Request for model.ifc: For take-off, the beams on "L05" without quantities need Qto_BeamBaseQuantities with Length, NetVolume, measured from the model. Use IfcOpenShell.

First a look at what the model holds.

```python
import ifcopenshell
import ifcopenshell.util.element
import ifcopenshell.util.unit

model = ifcopenshell.open("model.ifc")
print(model.schema)
for unit_type in ("LENGTHUNIT", "AREAUNIT", "VOLUMEUNIT"):
    print(unit_type, ifcopenshell.util.unit.calculate_unit_scale(model, unit_type))
storey = next(s for s in model.by_type("IfcBuildingStorey") if s.Name == "L05")
beams = [e for e in ifcopenshell.util.element.get_decomposition(storey) if e.is_a("IfcBeam")]
for e in sorted(beams, key=lambda e: e.id()):
    print(e.id(), e.is_a(), e.Name, list(ifcopenshell.util.element.get_psets(e, qtos_only=True)), sep=" | ")
```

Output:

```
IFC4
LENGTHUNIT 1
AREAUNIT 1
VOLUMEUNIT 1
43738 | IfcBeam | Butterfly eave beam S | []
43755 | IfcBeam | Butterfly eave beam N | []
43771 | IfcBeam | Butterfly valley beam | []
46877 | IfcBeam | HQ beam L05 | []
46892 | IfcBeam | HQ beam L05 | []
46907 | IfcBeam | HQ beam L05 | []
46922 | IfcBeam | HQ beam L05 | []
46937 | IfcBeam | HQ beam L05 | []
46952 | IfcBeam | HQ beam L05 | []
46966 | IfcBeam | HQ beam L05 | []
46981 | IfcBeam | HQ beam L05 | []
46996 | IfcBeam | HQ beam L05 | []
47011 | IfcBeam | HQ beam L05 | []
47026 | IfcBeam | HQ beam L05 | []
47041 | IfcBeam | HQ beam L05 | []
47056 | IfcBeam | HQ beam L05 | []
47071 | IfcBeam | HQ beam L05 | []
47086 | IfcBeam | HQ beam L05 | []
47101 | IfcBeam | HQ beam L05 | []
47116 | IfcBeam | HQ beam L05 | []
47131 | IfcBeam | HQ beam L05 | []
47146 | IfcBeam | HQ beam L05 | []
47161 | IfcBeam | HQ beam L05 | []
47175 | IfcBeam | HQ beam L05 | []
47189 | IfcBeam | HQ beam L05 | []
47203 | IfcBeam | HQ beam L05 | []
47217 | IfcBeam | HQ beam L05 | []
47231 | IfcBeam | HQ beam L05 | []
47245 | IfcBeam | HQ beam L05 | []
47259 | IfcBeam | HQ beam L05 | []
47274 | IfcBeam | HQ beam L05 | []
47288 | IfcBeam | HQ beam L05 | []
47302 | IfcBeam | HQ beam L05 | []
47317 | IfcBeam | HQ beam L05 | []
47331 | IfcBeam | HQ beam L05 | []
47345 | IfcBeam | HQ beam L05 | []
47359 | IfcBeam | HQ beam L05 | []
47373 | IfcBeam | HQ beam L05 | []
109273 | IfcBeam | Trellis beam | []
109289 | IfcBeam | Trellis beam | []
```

```python
import ifcopenshell
import ifcopenshell.api.pset
import ifcopenshell.geom
import ifcopenshell.util.element
import ifcopenshell.util.shape
import ifcopenshell.util.unit

model = ifcopenshell.open("model.ifc")
unit_scale = ifcopenshell.util.unit.calculate_unit_scale(model)
volume_scale = ifcopenshell.util.unit.calculate_unit_scale(model, "VOLUMEUNIT")
settings = ifcopenshell.geom.settings()

storey = next(s for s in model.by_type("IfcBuildingStorey") if s.Name == "L05")
beams = [e for e in ifcopenshell.util.element.get_decomposition(storey) if e.is_a("IfcBeam")]

for e in sorted(beams, key=lambda e: e.id()):
    if ifcopenshell.util.element.get_psets(e, qtos_only=True, should_inherit=False):
        continue
    # Geometry comes back in metres, in the element's own axes.
    shape = ifcopenshell.geom.create_shape(settings, e)
    values = {
        "Length": ifcopenshell.util.shape.get_max_xyz(shape.geometry) / unit_scale,
        "NetVolume": ifcopenshell.util.shape.get_volume(shape.geometry) / volume_scale,
    }
    qto = ifcopenshell.api.pset.add_qto(model, product=e, name="Qto_BeamBaseQuantities")
    ifcopenshell.api.pset.edit_qto(model, qto=qto, properties=values)
    print(e.id(), {k: round(v, 3) for k, v in values.items()})

model.write("model_updated.ifc")
```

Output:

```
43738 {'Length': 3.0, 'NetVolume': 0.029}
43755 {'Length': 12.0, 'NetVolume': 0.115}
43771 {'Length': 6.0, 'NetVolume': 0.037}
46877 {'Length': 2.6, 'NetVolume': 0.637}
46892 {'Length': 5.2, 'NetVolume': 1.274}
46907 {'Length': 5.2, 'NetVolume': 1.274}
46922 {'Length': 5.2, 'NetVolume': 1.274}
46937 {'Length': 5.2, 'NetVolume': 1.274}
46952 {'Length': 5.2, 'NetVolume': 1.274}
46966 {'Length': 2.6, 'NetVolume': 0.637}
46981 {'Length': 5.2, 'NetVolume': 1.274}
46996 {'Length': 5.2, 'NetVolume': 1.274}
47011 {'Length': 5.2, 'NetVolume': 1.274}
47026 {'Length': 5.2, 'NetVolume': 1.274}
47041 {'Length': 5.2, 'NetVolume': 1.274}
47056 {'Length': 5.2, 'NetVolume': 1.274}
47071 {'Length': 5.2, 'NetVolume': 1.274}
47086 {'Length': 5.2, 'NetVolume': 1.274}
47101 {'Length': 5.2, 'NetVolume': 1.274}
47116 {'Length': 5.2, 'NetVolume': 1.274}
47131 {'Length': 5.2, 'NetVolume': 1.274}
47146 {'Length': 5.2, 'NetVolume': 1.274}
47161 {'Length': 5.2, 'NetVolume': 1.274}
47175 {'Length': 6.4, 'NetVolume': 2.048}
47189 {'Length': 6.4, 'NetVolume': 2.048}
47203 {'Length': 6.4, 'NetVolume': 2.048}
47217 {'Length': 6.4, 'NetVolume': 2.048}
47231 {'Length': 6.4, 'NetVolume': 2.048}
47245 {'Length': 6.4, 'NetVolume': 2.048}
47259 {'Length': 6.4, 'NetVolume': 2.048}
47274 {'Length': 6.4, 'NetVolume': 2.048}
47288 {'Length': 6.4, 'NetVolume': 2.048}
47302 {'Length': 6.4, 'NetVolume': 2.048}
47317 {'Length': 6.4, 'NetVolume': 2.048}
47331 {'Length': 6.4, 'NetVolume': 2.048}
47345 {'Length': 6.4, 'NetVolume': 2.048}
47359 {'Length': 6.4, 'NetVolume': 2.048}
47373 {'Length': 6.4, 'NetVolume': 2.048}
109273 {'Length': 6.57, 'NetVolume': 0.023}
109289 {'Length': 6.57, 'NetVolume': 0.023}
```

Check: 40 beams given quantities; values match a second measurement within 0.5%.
